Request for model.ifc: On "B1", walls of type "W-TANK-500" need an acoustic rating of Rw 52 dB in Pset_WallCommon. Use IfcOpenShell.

First a look at what the model holds.

```python
import ifcopenshell
import ifcopenshell.util.element

model = ifcopenshell.open("model.ifc")
print(model.schema)
storey = next(s for s in model.by_type("IfcBuildingStorey") if s.Name == "B1")
walls = [e for e in ifcopenshell.util.element.get_decomposition(storey) if e.is_a("IfcWall")]
seen = {}
for e in walls:
    element_type = ifcopenshell.util.element.get_type(e)
    key = (element_type.Name if element_type != e and element_type else None, ifcopenshell.util.element.get_pset(e, "Pset_WallCommon", "AcousticRating"))
    seen[key] = seen.get(key, 0) + 1
for (name, value), count in sorted(seen.items(), key=str):
    print(count, "x", name, "|", value)
```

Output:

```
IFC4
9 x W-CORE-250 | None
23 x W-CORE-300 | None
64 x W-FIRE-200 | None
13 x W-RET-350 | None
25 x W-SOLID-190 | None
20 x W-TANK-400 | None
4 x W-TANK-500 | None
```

```python
import ifcopenshell
import ifcopenshell.api.pset
import ifcopenshell.util.element

model = ifcopenshell.open("model.ifc")

storey = next(s for s in model.by_type("IfcBuildingStorey") if s.Name == "B1")
walls = [e for e in ifcopenshell.util.element.get_decomposition(storey) if e.is_a("IfcWall")]

count = 0
for e in walls:
    element_type = ifcopenshell.util.element.get_type(e)
    if element_type in (None, e) or element_type.Name != "W-TANK-500":
        continue
    # add_pset returns the element's existing set when there is one.
    pset = ifcopenshell.api.pset.add_pset(model, product=e, name="Pset_WallCommon")
    ifcopenshell.api.pset.edit_pset(model, pset=pset, properties={"AcousticRating": "Rw 52 dB"})
    count += 1

print(count, "walls updated")

model.write("model_rev.ifc")
```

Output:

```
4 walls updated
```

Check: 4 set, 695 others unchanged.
